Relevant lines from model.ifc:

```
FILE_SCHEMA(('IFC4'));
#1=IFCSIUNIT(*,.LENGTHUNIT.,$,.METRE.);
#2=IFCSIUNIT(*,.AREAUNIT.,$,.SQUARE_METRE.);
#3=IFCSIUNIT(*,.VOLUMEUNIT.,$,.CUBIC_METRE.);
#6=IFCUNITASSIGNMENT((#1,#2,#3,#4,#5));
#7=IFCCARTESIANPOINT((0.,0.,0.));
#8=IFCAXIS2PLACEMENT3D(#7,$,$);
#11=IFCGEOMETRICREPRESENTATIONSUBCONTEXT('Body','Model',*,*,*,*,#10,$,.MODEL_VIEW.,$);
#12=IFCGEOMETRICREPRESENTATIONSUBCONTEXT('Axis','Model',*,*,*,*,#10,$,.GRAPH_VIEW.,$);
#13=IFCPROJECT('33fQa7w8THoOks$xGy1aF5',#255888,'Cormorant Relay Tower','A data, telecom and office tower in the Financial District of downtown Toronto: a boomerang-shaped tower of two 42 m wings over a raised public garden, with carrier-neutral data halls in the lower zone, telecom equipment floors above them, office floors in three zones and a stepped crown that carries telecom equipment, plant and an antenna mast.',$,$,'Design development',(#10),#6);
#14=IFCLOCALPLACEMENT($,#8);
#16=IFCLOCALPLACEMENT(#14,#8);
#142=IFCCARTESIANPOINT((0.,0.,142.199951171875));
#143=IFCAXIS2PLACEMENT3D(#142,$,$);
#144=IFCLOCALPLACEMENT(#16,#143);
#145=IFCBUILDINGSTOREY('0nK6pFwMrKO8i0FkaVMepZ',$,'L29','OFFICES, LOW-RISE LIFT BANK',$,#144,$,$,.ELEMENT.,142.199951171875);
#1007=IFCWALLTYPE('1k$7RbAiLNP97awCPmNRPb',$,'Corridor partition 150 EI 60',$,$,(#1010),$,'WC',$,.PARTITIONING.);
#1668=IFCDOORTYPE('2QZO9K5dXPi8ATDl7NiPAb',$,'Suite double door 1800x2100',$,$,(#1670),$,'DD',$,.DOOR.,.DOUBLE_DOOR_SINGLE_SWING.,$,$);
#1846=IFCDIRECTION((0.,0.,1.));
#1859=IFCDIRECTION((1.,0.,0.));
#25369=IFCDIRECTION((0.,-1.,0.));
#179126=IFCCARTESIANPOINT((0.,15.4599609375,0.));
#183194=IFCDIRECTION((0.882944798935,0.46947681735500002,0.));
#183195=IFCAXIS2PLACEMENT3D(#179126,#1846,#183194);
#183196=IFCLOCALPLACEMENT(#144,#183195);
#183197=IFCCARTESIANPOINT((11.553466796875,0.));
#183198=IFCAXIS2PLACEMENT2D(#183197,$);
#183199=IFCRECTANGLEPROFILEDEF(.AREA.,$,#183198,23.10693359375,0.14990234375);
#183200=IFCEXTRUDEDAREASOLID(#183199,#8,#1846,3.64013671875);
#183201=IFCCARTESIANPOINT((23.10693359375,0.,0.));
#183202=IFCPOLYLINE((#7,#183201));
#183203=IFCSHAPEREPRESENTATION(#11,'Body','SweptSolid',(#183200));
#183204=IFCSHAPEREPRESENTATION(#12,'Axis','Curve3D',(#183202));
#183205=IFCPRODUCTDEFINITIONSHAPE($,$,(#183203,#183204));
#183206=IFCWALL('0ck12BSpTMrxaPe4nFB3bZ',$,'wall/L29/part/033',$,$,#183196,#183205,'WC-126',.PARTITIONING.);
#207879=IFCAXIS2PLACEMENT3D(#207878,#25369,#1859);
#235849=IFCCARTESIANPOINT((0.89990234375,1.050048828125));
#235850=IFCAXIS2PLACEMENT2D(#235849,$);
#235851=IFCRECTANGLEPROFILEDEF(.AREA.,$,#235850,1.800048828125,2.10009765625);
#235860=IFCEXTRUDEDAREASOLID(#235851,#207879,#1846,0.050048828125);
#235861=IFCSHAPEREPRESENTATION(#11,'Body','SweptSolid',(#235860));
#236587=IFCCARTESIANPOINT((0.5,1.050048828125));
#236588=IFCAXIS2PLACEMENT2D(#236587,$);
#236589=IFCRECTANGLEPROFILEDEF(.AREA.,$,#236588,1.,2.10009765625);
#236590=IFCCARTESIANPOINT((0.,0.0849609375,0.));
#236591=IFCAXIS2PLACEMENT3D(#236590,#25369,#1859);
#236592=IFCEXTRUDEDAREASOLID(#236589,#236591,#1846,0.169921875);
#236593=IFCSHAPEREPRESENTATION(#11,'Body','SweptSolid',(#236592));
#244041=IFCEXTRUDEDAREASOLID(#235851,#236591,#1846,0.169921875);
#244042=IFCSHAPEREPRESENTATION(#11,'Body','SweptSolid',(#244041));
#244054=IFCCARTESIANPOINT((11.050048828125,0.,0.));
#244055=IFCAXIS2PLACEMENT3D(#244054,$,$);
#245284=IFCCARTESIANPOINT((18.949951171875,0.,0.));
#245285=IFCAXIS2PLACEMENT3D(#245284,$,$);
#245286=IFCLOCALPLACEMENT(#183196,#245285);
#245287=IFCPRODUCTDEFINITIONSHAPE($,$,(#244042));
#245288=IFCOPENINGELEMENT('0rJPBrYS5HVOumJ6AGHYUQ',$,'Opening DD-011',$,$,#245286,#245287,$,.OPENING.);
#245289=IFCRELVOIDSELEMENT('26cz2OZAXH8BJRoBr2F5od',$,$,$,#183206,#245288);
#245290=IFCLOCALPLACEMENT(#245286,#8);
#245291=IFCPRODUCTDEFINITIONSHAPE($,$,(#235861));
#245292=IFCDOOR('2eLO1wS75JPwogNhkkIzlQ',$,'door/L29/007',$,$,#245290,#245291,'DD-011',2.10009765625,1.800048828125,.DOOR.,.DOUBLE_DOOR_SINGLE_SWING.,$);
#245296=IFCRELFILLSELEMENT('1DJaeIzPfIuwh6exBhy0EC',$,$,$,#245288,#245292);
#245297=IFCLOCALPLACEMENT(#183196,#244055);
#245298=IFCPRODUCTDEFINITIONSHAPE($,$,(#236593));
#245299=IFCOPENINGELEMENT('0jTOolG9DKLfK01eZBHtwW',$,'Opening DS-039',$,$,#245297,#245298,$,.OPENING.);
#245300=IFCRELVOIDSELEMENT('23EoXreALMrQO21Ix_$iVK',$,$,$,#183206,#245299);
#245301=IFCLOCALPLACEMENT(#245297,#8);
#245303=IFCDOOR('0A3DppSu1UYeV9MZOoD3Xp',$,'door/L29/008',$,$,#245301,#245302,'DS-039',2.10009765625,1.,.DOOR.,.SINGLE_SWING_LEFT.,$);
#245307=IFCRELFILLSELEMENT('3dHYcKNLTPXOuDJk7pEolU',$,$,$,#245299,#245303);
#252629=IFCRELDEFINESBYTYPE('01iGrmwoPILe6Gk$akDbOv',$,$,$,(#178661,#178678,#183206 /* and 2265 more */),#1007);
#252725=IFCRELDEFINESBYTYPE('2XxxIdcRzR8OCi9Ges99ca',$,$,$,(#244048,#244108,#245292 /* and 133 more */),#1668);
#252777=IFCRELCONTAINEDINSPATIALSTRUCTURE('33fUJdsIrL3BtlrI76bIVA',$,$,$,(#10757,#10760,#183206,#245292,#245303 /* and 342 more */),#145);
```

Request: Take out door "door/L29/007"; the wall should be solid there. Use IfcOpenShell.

```python
import ifcopenshell
import ifcopenshell.api.feature
import ifcopenshell.api.root
import ifcopenshell.geom
import ifcopenshell.util.shape

model = ifcopenshell.open("model.ifc")
settings = ifcopenshell.geom.settings()


def volume(element):
    """Net volume in cubic metres, openings subtracted."""
    shape = ifcopenshell.geom.create_shape(settings, element)
    return ifcopenshell.util.shape.get_volume(shape.geometry)


door = model.by_guid("2eLO1wS75JPwogNhkkIzlQ")
opening = door.FillsVoids[0].RelatingOpeningElement
wall = opening.VoidsElements[0].RelatingBuildingElement
before = volume(wall)

ifcopenshell.api.root.remove_product(model, product=door)
ifcopenshell.api.feature.remove_feature(model, feature=opening)

after = volume(wall)

print(f"wall volume {before:.3f} -> {after:.3f} m3")

model.write("model_edited.ifc")
```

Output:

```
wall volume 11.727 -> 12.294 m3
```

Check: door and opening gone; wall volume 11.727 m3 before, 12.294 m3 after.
